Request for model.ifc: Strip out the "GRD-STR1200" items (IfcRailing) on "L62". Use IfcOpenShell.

First a look at what the model holds.

```python
import ifcopenshell
import ifcopenshell.util.element

model = ifcopenshell.open("model.ifc")
print(model.schema)
storey = next(s for s in model.by_type("IfcBuildingStorey") if s.Name == "L62")
railings = [e for e in ifcopenshell.util.element.get_decomposition(storey) if e.is_a("IfcRailing")]
seen = {}
for e in railings:
    element_type = ifcopenshell.util.element.get_type(e)
    name = element_type.Name if element_type not in (None, e) else None
    seen[name] = seen.get(name, 0) + 1
for name, count in sorted(seen.items(), key=str):
    print(count, "x", name)
```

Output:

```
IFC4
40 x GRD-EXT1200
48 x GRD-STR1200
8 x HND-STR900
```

```python
import ifcopenshell
import ifcopenshell.api.root
import ifcopenshell.util.element

model = ifcopenshell.open("model.ifc")

storey = next(s for s in model.by_type("IfcBuildingStorey") if s.Name == "L62")
railings = [e for e in ifcopenshell.util.element.get_decomposition(storey) if e.is_a("IfcRailing")]
targets = [e for e in railings if (t := ifcopenshell.util.element.get_type(e)) not in (None, e) and t.Name == "GRD-STR1200"]

for e in targets:
    ifcopenshell.api.root.remove_product(model, product=e)
print(len(targets), "removed")

model.write("model_updated.ifc")
```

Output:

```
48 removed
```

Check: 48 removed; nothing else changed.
